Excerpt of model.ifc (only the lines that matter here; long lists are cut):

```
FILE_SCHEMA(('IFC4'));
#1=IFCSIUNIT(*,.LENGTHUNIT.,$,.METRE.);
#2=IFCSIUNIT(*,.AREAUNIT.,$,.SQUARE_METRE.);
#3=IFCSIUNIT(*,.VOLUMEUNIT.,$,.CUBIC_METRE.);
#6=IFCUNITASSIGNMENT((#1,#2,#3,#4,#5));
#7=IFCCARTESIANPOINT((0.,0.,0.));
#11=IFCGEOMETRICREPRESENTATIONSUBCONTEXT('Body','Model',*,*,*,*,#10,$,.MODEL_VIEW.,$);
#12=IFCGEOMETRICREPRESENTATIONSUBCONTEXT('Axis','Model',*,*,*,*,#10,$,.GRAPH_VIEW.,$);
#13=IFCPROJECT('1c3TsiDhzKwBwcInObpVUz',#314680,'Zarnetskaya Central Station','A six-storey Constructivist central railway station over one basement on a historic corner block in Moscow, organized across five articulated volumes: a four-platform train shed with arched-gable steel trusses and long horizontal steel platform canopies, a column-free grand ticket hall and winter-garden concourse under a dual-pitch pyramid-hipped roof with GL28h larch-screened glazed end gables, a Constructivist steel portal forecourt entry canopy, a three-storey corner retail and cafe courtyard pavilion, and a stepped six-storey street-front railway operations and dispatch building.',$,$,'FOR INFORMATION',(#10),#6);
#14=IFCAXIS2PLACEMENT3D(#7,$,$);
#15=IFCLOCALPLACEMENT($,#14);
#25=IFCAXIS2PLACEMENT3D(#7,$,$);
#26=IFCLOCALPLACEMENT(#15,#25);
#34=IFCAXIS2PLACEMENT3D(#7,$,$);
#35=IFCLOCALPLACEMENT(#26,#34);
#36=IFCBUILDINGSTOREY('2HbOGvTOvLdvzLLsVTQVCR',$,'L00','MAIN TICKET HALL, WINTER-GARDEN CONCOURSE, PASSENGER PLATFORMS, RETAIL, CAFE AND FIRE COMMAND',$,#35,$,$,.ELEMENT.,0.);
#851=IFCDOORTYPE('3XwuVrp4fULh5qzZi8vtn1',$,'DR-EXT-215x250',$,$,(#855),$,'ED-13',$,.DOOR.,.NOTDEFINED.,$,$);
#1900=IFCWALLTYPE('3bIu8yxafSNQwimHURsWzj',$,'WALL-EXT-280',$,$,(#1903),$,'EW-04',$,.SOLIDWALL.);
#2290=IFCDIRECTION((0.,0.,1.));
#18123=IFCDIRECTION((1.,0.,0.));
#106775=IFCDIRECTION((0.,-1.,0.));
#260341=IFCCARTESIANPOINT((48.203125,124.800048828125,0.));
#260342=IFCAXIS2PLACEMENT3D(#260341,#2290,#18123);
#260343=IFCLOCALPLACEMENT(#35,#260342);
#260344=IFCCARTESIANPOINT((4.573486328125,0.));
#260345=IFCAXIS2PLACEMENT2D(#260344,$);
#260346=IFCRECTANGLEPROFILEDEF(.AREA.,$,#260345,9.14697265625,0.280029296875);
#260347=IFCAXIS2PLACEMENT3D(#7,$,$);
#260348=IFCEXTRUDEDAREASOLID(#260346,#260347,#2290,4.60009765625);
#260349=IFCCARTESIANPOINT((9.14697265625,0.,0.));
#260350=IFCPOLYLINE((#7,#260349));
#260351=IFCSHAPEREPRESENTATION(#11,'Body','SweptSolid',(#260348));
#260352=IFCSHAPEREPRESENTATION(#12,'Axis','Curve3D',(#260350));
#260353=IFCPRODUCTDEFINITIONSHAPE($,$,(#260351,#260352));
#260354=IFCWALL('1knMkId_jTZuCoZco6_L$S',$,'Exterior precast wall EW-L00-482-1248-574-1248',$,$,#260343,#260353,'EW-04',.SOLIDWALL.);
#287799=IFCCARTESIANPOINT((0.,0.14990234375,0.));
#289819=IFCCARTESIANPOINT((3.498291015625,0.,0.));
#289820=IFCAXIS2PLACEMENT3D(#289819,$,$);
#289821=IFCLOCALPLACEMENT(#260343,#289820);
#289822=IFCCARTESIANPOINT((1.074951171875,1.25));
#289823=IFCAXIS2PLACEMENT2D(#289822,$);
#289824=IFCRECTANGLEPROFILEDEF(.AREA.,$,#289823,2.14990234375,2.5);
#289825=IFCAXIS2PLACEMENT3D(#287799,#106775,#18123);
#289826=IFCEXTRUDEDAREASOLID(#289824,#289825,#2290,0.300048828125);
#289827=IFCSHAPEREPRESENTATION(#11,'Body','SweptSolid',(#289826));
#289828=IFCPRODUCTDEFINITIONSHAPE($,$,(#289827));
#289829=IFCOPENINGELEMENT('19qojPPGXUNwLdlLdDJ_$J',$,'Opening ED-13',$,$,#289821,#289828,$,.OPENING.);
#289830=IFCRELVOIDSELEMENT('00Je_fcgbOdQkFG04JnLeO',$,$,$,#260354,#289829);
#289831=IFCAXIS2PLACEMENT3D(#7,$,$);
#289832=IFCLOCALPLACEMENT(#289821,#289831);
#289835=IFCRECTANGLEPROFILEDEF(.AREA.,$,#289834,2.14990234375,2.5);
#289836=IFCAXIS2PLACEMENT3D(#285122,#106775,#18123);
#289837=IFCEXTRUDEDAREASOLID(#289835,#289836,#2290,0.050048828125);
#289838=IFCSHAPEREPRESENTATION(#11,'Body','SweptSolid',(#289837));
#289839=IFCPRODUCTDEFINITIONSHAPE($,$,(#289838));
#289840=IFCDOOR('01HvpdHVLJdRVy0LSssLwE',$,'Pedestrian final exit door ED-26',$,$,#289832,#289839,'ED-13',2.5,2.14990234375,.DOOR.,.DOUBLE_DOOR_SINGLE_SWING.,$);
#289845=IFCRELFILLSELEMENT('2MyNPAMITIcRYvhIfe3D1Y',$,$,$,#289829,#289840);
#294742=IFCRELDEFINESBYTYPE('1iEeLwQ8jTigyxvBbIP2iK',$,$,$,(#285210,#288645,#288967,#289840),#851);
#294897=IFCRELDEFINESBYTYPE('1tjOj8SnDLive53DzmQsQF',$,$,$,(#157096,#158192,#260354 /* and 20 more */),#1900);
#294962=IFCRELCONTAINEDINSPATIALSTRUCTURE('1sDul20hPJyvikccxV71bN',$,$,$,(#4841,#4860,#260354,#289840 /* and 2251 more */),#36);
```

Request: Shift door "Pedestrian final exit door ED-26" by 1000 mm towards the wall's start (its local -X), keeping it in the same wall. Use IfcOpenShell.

```python
import ifcopenshell
import ifcopenshell.api.geometry
import ifcopenshell.util.placement

model = ifcopenshell.open("model.ifc")

door = model.by_id(289840)
opening = door.FillsVoids[0].RelatingOpeningElement
wall = opening.VoidsElements[0].RelatingBuildingElement

wall_matrix = ifcopenshell.util.placement.get_local_placement(wall.ObjectPlacement)
shift = wall_matrix[:3, 0] * -1.0
before = ifcopenshell.util.placement.get_local_placement(door.ObjectPlacement)[:3, 3].copy()

# The door is placed relative to its opening, so it follows when the opening moves.
matrix = ifcopenshell.util.placement.get_local_placement(opening.ObjectPlacement)
matrix[:3, 3] += shift
ifcopenshell.api.geometry.edit_object_placement(
    model, product=opening, matrix=matrix, is_si=False, should_transform_children=True
)

after = ifcopenshell.util.placement.get_local_placement(door.ObjectPlacement)[:3, 3]
print("door moved by", (after - before).round(3) + 0.0)

model.write("model_updated.ifc")
```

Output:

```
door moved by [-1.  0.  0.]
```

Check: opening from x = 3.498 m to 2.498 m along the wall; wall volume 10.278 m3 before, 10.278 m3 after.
